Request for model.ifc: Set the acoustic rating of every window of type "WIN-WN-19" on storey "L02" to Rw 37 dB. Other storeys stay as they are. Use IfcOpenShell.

First a look at what the model holds.

```python
import ifcopenshell
import ifcopenshell.util.element

model = ifcopenshell.open("model.ifc")
print(model.schema)
storey = next(s for s in model.by_type("IfcBuildingStorey") if s.Name == "L02")
windows = [e for e in ifcopenshell.util.element.get_decomposition(storey) if e.is_a("IfcWindow")]
seen = {}
for e in windows:
    element_type = ifcopenshell.util.element.get_type(e)
    key = (element_type.Name if element_type != e and element_type else None, ifcopenshell.util.element.get_pset(e, "Pset_WindowCommon", "AcousticRating"))
    seen[key] = seen.get(key, 0) + 1
for (name, value), count in sorted(seen.items(), key=str):
    print(count, "x", name, "|", value)
```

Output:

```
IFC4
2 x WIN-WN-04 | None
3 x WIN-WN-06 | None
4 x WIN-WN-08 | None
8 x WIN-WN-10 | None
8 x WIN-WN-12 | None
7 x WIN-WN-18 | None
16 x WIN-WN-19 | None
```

```python
import ifcopenshell
import ifcopenshell.api.pset
import ifcopenshell.util.element

model = ifcopenshell.open("model.ifc")

storey = next(s for s in model.by_type("IfcBuildingStorey") if s.Name == "L02")
windows = [e for e in ifcopenshell.util.element.get_decomposition(storey) if e.is_a("IfcWindow")]

count = 0
for e in windows:
    element_type = ifcopenshell.util.element.get_type(e)
    if element_type in (None, e) or element_type.Name != "WIN-WN-19":
        continue
    # add_pset returns the element's existing set when there is one.
    pset = ifcopenshell.api.pset.add_pset(model, product=e, name="Pset_WindowCommon")
    ifcopenshell.api.pset.edit_pset(model, pset=pset, properties={"AcousticRating": "Rw 37 dB"})
    count += 1

print(count, "windows updated")

model.write("model_edited.ifc")
```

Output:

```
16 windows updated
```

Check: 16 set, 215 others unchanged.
